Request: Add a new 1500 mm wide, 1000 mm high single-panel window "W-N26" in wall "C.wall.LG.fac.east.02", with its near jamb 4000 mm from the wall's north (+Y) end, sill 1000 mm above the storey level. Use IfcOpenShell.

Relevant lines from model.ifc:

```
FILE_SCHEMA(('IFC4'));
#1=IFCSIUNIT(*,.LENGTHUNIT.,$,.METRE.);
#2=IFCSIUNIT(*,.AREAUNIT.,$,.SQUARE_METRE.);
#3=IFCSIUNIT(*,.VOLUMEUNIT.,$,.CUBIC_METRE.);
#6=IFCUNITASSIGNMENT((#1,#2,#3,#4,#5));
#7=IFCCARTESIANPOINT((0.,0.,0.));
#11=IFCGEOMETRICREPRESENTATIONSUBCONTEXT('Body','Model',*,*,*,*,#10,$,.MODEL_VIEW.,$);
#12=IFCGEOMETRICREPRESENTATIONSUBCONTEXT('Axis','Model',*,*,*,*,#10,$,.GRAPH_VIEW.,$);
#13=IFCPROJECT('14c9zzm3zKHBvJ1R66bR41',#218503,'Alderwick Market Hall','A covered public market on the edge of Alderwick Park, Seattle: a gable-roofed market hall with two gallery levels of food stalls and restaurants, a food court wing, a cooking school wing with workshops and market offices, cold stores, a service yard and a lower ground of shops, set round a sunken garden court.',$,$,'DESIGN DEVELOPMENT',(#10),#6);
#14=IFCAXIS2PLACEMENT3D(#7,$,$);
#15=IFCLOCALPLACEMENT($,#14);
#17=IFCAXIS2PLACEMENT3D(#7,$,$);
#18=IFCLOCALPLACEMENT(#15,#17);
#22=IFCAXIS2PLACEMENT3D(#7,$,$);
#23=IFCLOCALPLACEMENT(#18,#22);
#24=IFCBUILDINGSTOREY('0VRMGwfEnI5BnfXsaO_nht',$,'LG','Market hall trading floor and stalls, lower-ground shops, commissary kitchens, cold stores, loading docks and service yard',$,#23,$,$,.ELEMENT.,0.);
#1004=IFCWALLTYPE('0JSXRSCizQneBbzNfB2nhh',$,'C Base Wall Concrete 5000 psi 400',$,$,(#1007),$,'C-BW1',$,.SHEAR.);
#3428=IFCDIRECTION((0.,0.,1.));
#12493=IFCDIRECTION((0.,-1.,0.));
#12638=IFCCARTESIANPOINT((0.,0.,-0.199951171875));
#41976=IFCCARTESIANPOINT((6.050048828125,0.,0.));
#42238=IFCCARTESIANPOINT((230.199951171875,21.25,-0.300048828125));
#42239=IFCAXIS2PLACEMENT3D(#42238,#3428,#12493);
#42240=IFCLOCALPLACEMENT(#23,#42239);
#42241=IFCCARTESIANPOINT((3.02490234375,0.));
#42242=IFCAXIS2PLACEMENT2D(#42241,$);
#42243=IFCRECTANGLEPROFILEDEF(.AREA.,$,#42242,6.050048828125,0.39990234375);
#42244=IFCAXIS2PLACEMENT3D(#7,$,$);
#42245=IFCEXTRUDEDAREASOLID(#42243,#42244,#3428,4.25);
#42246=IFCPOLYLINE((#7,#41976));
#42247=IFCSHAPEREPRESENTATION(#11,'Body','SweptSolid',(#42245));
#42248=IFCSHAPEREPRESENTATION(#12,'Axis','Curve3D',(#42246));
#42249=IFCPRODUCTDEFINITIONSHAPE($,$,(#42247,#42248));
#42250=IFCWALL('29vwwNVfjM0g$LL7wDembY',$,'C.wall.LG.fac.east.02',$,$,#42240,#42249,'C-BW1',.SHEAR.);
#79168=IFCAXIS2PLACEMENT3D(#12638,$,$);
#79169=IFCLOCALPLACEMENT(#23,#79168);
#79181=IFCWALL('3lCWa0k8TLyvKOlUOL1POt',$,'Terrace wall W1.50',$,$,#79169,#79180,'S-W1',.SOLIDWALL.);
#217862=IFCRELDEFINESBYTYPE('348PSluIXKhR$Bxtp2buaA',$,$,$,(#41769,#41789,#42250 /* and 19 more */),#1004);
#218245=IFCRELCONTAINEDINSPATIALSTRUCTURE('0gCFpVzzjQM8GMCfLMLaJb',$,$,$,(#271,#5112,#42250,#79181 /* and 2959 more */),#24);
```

```python
import numpy as np
import ifcopenshell
import ifcopenshell.api.feature
import ifcopenshell.api.geometry
import ifcopenshell.api.root
import ifcopenshell.api.spatial
import ifcopenshell.geom
import ifcopenshell.util.element
import ifcopenshell.util.placement
import ifcopenshell.util.representation
import ifcopenshell.util.shape
import ifcopenshell.util.unit

model = ifcopenshell.open("model.ifc")
unit_scale = ifcopenshell.util.unit.calculate_unit_scale(model)
settings = ifcopenshell.geom.settings()


def volume(element):
    """Net volume in cubic metres, openings subtracted."""
    shape = ifcopenshell.geom.create_shape(settings, element)
    return ifcopenshell.util.shape.get_volume(shape.geometry)


wall = model.by_guid("29vwwNVfjM0g$LL7wDembY")
storey = ifcopenshell.util.element.get_container(wall, ifc_class="IfcBuildingStorey")
context = ifcopenshell.util.representation.get_context(model, "Model", "Body", "MODEL_VIEW")
before = volume(wall)

width, height, from_end, sill = 1.5, 1, 4, 1  # metres

# The wall runs along its own X axis, and the end named is its -X end.
wall_shape = ifcopenshell.geom.create_shape(settings, wall)
x, y, z = ifcopenshell.util.shape.get_vertices(wall_shape.geometry).T
start = x.min() + from_end
face, thickness = float(y.min()), float(y.max() - y.min())
wall_matrix = ifcopenshell.util.placement.get_local_placement(wall.ObjectPlacement)
level = ifcopenshell.util.placement.get_local_placement(storey.ObjectPlacement)[2, 3]


def in_wall(x, y):
    """Placement at x, y metres in the wall's axes, at sill height."""
    matrix = wall_matrix.copy()
    matrix[:, 3] = wall_matrix @ np.array([x / unit_scale, y / unit_scale, 0.0, 1.0])
    matrix[2, 3] = level + sill / unit_scale
    return matrix


# Opening: a box that overshoots both wall faces by 50 mm.
opening = ifcopenshell.api.root.create_entity(model, ifc_class="IfcOpeningElement", predefined_type="OPENING")
box = ifcopenshell.api.geometry.add_wall_representation(
    model, context=context, length=width, height=height, thickness=thickness + 0.1
)
ifcopenshell.api.geometry.assign_representation(model, product=opening, representation=box)
ifcopenshell.api.geometry.edit_object_placement(model, product=opening, matrix=in_wall(start, face - 0.05), is_si=False)
ifcopenshell.api.feature.add_feature(model, feature=opening, element=wall)

window = ifcopenshell.api.root.create_entity(model, ifc_class="IfcWindow", name="W-N26", predefined_type="WINDOW")
window.OverallWidth, window.OverallHeight = width / unit_scale, height / unit_scale
window.PartitioningType = "SINGLE_PANEL"
body = ifcopenshell.api.geometry.add_window_representation(
    model,
    context=context,
    overall_width=window.OverallWidth,
    overall_height=window.OverallHeight,
    partition_type="SINGLE_PANEL",
)
ifcopenshell.api.geometry.assign_representation(model, product=window, representation=body)
ifcopenshell.api.spatial.assign_container(model, products=[window], relating_structure=storey)
ifcopenshell.api.feature.add_filling(model, opening=opening, element=window)

# Centre the window in the wall's thickness.
ifcopenshell.api.geometry.edit_object_placement(model, product=window, matrix=in_wall(start, face), is_si=False)
window_shape = ifcopenshell.geom.create_shape(settings, window)
depth = ifcopenshell.util.shape.get_vertices(window_shape.geometry)[:, 1]
offset = face + thickness / 2 - (depth.min() + depth.max()) / 2
ifcopenshell.api.geometry.edit_object_placement(model, product=window, matrix=in_wall(start, offset), is_si=False)

after = volume(wall)

print(f"wall volume {before:.3f} -> {after:.3f} m3")

model.write("model-out.ifc")
```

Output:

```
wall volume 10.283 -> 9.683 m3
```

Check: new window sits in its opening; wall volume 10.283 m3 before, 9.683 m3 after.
